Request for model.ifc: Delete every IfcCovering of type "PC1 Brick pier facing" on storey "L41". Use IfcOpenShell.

First a look at what the model holds.

```python
import ifcopenshell
import ifcopenshell.util.element

model = ifcopenshell.open("model.ifc")
print(model.schema)
storey = next(s for s in model.by_type("IfcBuildingStorey") if s.Name == "L41")
coverings = [e for e in ifcopenshell.util.element.get_decomposition(storey) if e.is_a("IfcCovering")]
seen = {}
for e in coverings:
    element_type = ifcopenshell.util.element.get_type(e)
    name = element_type.Name if element_type not in (None, e) else None
    seen[name] = seen.get(name, 0) + 1
for name, count in sorted(seen.items(), key=str):
    print(count, "x", name)
```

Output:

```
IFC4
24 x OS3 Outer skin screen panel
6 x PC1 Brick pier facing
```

```python
import ifcopenshell
import ifcopenshell.api.root
import ifcopenshell.util.element

model = ifcopenshell.open("model.ifc")

storey = next(s for s in model.by_type("IfcBuildingStorey") if s.Name == "L41")
coverings = [e for e in ifcopenshell.util.element.get_decomposition(storey) if e.is_a("IfcCovering")]
targets = [e for e in coverings if (t := ifcopenshell.util.element.get_type(e)) not in (None, e) and t.Name == "PC1 Brick pier facing"]

for e in targets:
    ifcopenshell.api.root.remove_product(model, product=e)
print(len(targets), "removed")

model.write("model-out.ifc")
```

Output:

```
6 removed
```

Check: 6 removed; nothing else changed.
